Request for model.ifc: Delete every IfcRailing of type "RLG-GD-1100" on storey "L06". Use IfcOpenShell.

First a look at what the model holds.

```python
import ifcopenshell
import ifcopenshell.util.element

model = ifcopenshell.open("model.ifc")
print(model.schema)
storey = next(s for s in model.by_type("IfcBuildingStorey") if s.Name == "L06")
railings = [e for e in ifcopenshell.util.element.get_decomposition(storey) if e.is_a("IfcRailing")]
seen = {}
for e in railings:
    element_type = ifcopenshell.util.element.get_type(e)
    name = element_type.Name if element_type not in (None, e) else None
    seen[name] = seen.get(name, 0) + 1
for name, count in sorted(seen.items(), key=str):
    print(count, "x", name)
```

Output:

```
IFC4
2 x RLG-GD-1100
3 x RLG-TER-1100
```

```python
import ifcopenshell
import ifcopenshell.api.root
import ifcopenshell.util.element

model = ifcopenshell.open("model.ifc")

storey = next(s for s in model.by_type("IfcBuildingStorey") if s.Name == "L06")
railings = [e for e in ifcopenshell.util.element.get_decomposition(storey) if e.is_a("IfcRailing")]
targets = [e for e in railings if (t := ifcopenshell.util.element.get_type(e)) not in (None, e) and t.Name == "RLG-GD-1100"]

for e in targets:
    ifcopenshell.api.root.remove_product(model, product=e)
print(len(targets), "removed")

model.write("model_rev.ifc")
```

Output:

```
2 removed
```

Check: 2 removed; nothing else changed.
